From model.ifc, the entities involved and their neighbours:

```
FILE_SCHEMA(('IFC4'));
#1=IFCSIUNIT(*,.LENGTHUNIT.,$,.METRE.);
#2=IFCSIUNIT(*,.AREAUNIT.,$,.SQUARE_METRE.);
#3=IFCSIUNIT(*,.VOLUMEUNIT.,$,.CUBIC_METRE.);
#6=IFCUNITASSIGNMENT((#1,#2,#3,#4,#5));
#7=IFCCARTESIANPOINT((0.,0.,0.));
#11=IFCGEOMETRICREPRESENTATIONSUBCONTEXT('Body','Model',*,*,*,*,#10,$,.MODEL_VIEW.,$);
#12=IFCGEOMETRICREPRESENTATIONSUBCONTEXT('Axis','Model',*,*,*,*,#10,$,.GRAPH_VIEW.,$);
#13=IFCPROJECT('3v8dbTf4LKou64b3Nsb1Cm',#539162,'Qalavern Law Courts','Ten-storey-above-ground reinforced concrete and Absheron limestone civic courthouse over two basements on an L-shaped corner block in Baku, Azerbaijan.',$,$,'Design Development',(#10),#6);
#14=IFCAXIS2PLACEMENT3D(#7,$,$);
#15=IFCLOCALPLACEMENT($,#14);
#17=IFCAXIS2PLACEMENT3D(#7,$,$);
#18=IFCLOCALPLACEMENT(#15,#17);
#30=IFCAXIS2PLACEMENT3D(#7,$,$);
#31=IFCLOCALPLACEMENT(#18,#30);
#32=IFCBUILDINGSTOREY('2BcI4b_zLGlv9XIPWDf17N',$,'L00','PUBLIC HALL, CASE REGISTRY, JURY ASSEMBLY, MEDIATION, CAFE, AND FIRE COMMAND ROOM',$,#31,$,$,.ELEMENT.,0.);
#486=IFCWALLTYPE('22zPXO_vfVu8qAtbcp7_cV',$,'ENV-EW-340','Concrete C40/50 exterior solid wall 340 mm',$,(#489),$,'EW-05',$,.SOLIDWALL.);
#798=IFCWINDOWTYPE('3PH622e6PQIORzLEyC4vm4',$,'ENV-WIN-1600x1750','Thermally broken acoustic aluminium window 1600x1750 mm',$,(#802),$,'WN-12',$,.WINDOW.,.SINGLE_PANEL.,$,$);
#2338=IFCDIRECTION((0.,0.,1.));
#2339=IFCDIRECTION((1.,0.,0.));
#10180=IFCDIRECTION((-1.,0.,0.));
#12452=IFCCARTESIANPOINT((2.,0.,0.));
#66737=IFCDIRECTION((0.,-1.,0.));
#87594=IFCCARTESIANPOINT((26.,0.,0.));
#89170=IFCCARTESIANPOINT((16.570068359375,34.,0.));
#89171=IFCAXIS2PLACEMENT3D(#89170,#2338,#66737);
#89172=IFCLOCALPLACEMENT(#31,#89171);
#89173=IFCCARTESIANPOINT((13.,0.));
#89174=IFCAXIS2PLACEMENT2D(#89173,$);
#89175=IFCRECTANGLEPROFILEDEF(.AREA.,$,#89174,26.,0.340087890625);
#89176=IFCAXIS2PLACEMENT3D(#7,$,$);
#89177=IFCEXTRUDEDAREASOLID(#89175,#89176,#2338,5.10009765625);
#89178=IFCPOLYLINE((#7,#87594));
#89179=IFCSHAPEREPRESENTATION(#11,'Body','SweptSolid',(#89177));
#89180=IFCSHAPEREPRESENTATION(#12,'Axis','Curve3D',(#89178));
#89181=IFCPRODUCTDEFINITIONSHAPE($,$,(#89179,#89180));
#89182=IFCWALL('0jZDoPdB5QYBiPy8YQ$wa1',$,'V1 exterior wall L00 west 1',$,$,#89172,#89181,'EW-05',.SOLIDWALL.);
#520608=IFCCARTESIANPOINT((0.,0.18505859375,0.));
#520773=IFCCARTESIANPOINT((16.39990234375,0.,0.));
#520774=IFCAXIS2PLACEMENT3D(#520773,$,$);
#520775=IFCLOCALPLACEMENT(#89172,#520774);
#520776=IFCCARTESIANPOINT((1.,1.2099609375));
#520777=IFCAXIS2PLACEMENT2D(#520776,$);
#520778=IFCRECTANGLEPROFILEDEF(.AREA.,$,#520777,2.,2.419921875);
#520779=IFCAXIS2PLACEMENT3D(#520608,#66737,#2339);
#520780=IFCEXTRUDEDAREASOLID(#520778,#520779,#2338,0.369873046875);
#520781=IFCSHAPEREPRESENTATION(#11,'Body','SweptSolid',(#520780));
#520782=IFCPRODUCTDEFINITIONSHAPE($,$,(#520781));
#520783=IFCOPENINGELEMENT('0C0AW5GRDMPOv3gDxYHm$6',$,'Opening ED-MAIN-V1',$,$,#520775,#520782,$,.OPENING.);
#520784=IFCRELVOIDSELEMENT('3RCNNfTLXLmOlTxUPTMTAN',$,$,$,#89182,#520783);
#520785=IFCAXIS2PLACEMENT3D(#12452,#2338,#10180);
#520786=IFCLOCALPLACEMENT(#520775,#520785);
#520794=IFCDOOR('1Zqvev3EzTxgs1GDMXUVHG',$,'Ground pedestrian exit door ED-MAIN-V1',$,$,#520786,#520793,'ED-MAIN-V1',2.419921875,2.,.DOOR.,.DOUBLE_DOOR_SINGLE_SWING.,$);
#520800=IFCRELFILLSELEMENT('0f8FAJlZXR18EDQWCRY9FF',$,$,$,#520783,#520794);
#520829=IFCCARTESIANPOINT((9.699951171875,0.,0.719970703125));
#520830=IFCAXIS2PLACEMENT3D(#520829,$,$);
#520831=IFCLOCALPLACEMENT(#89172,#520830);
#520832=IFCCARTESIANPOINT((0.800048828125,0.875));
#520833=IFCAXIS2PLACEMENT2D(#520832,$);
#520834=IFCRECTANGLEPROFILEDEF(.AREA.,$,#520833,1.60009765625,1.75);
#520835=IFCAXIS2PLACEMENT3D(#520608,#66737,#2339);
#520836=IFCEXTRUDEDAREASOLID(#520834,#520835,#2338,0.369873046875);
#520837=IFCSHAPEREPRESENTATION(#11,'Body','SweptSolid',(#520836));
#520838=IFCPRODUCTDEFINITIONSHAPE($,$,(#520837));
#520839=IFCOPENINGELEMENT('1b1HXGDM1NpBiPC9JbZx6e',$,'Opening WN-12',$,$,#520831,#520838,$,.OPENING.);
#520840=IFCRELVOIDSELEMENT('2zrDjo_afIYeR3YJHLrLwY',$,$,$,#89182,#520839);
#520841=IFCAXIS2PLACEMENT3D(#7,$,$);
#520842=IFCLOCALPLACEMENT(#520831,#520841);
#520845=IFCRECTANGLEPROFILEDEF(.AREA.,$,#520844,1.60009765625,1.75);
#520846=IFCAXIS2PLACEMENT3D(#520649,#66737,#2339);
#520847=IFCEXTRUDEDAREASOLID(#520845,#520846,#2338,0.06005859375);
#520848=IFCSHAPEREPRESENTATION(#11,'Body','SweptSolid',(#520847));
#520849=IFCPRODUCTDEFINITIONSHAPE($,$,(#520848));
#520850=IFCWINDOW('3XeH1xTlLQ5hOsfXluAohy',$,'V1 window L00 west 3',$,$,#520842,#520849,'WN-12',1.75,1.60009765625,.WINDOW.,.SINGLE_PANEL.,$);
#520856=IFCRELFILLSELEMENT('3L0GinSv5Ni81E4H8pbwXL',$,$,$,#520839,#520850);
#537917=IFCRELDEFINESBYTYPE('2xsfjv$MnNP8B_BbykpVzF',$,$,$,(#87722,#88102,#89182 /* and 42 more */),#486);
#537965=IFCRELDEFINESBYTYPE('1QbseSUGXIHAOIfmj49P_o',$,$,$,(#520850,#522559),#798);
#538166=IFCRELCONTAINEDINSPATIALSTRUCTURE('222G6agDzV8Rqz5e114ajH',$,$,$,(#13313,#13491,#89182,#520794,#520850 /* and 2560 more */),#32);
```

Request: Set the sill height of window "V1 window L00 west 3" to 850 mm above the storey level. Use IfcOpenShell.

```python
import numpy as np
import ifcopenshell
import ifcopenshell.api.geometry
import ifcopenshell.geom
import ifcopenshell.util.element
import ifcopenshell.util.placement
import ifcopenshell.util.shape
import ifcopenshell.util.unit

model = ifcopenshell.open("model.ifc")
unit_scale = ifcopenshell.util.unit.calculate_unit_scale(model)

window = model.by_guid("3XeH1xTlLQ5hOsfXluAohy")
opening = window.FillsVoids[0].RelatingOpeningElement
storey = ifcopenshell.util.element.get_container(window, ifc_class="IfcBuildingStorey")
level = ifcopenshell.util.placement.get_local_placement(storey.ObjectPlacement)[2, 3]

# The opening's origin need not be at the sill, so measure its lowest point.
shape = ifcopenshell.geom.create_shape(ifcopenshell.geom.settings(), opening)
bottom = ifcopenshell.util.shape.get_shape_bottom_elevation(shape, shape.geometry) / unit_scale
dz = level + 0.85 / unit_scale - bottom

shift = np.array([0.0, 0.0, dz])
# The window is placed relative to its opening, so it follows when the opening moves.
matrix = ifcopenshell.util.placement.get_local_placement(opening.ObjectPlacement)
matrix[:3, 3] += shift
ifcopenshell.api.geometry.edit_object_placement(
    model, product=opening, matrix=matrix, is_si=False, should_transform_children=True
)

print(f"moved by {dz * unit_scale:+.3f} m")

model.write("model_rev.ifc")
```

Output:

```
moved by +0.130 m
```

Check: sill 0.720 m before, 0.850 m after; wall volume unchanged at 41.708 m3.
